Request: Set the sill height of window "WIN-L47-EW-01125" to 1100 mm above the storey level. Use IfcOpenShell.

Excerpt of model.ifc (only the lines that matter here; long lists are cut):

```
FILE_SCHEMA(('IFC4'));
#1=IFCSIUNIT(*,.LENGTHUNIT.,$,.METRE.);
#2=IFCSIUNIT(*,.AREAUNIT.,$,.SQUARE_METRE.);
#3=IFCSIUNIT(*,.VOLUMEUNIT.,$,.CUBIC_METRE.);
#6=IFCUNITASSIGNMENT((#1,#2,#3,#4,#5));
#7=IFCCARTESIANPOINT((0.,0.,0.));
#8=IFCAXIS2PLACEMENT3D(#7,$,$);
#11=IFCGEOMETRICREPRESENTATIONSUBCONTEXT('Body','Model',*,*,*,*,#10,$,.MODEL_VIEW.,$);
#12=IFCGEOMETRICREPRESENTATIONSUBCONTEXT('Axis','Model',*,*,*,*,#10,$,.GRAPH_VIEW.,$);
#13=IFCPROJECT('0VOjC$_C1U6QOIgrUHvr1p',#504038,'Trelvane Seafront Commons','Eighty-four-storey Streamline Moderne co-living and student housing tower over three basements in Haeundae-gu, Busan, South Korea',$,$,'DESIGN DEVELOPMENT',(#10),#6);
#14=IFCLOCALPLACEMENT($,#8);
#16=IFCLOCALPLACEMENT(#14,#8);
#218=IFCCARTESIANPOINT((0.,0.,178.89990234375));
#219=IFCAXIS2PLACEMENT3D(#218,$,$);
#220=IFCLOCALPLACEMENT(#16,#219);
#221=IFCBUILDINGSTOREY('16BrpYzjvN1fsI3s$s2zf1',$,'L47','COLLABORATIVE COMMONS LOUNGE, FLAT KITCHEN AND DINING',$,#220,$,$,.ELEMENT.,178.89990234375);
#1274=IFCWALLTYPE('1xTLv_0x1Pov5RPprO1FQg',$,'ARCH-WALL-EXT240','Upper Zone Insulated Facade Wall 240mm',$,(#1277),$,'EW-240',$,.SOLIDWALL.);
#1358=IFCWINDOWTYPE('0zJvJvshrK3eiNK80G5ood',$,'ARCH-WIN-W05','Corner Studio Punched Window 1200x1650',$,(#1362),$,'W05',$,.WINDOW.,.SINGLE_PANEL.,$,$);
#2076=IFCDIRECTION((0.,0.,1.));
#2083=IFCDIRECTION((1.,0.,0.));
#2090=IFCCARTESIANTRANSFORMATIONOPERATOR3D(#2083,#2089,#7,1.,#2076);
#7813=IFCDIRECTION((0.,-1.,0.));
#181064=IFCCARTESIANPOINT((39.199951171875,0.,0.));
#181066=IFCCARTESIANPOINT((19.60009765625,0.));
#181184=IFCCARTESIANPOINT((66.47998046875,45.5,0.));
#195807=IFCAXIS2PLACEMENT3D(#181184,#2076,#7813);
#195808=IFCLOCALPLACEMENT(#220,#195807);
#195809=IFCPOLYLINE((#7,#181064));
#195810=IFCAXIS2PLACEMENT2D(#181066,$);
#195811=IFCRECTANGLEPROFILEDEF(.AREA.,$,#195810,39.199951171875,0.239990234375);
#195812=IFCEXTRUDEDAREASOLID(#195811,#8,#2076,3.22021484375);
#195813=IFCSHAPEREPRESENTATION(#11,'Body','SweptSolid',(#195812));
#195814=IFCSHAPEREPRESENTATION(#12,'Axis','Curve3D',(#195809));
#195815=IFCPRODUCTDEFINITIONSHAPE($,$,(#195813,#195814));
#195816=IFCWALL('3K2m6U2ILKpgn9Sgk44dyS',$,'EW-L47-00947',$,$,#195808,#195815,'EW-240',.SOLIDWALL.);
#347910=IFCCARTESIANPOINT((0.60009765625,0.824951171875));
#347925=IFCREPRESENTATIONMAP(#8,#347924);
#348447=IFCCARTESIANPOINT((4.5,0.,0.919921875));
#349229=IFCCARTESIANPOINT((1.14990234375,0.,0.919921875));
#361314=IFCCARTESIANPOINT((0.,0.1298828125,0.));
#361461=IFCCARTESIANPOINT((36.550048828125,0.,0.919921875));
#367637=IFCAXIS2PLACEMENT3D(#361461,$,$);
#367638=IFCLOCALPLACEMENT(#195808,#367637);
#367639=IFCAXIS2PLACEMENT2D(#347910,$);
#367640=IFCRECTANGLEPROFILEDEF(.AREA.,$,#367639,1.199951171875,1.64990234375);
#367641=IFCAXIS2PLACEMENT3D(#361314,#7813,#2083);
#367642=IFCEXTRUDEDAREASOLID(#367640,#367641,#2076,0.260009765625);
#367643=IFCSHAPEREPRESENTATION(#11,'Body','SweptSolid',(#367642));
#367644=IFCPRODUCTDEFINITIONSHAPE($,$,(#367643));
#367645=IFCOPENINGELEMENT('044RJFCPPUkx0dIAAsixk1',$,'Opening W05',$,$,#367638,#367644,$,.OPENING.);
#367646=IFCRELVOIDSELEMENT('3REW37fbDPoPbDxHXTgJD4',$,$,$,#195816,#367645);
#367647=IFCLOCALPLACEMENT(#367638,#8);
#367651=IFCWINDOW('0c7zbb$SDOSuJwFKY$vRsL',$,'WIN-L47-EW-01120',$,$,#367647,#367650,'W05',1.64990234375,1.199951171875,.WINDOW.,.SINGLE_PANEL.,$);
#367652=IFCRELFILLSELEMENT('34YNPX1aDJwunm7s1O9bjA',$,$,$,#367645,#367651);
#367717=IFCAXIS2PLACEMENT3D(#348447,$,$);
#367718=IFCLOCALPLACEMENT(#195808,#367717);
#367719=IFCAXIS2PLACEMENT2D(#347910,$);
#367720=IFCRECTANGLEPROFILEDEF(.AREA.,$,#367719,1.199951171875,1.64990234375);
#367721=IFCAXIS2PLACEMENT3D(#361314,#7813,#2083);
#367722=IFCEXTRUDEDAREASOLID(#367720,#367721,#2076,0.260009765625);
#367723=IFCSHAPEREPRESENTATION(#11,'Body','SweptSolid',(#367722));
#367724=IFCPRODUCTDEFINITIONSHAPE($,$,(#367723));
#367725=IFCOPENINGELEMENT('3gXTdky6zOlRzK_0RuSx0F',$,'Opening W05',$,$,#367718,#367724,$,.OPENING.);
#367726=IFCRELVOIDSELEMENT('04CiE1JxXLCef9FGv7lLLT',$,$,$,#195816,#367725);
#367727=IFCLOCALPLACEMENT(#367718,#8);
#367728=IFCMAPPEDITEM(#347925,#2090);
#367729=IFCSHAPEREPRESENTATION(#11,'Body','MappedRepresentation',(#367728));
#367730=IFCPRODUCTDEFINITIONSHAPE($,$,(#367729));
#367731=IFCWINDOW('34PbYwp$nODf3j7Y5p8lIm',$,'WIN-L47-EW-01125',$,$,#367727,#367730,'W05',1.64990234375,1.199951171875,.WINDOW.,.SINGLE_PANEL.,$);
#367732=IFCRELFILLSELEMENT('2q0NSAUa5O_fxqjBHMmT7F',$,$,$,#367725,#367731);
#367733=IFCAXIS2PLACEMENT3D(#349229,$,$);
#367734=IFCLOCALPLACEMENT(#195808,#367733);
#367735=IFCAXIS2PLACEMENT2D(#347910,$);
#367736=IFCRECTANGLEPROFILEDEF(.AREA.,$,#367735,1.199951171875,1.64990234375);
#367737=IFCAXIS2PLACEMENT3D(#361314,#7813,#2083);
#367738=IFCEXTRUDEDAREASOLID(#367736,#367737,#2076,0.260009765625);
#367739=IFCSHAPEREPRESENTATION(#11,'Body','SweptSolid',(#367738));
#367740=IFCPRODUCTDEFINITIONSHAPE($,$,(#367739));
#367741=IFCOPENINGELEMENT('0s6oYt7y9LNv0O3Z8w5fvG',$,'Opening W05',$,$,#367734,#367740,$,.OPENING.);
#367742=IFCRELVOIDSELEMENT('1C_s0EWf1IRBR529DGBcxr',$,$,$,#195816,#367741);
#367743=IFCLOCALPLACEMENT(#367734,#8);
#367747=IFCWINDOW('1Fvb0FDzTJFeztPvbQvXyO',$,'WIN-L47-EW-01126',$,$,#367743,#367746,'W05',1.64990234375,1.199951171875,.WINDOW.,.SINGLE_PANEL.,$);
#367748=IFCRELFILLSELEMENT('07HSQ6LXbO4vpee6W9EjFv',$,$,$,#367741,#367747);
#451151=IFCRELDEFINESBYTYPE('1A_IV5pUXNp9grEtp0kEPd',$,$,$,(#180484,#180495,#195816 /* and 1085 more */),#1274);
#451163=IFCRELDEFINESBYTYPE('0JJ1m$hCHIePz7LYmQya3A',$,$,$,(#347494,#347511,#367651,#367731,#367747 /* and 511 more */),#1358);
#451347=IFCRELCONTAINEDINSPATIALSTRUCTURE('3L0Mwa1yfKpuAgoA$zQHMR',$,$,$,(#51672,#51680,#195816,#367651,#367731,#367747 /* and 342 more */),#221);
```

```python
import numpy as np
import ifcopenshell
import ifcopenshell.api.geometry
import ifcopenshell.geom
import ifcopenshell.util.element
import ifcopenshell.util.placement
import ifcopenshell.util.shape
import ifcopenshell.util.unit

model = ifcopenshell.open("model.ifc")
unit_scale = ifcopenshell.util.unit.calculate_unit_scale(model)

window = model.by_guid("34PbYwp$nODf3j7Y5p8lIm")
opening = window.FillsVoids[0].RelatingOpeningElement
storey = ifcopenshell.util.element.get_container(window, ifc_class="IfcBuildingStorey")
level = ifcopenshell.util.placement.get_local_placement(storey.ObjectPlacement)[2, 3]

# The opening's origin need not be at the sill, so measure its lowest point.
shape = ifcopenshell.geom.create_shape(ifcopenshell.geom.settings(), opening)
bottom = ifcopenshell.util.shape.get_shape_bottom_elevation(shape, shape.geometry) / unit_scale
dz = level + 1.1 - bottom

shift = np.array([0.0, 0.0, dz])
# The window is placed relative to its opening, so it follows when the opening moves.
matrix = ifcopenshell.util.placement.get_local_placement(opening.ObjectPlacement)
matrix[:3, 3] += shift
ifcopenshell.api.geometry.edit_object_placement(
    model, product=opening, matrix=matrix, is_si=False, should_transform_children=True
)

print(f"moved by {dz * unit_scale:+.3f} m")

model.write("model-out.ifc")
```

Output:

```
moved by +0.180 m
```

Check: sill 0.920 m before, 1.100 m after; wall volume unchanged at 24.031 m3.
